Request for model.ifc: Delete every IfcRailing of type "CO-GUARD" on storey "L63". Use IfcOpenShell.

First a look at what the model holds.

```python
import ifcopenshell
import ifcopenshell.util.element

model = ifcopenshell.open("model.ifc")
print(model.schema)
storey = next(s for s in model.by_type("IfcBuildingStorey") if s.Name == "L63")
railings = [e for e in ifcopenshell.util.element.get_decomposition(storey) if e.is_a("IfcRailing")]
seen = {}
for e in railings:
    element_type = ifcopenshell.util.element.get_type(e)
    name = element_type.Name if element_type not in (None, e) else None
    seen[name] = seen.get(name, 0) + 1
for name, count in sorted(seen.items(), key=str):
    print(count, "x", name)
```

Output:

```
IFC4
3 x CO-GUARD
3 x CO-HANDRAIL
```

```python
import ifcopenshell
import ifcopenshell.api.root
import ifcopenshell.util.element

model = ifcopenshell.open("model.ifc")

storey = next(s for s in model.by_type("IfcBuildingStorey") if s.Name == "L63")
railings = [e for e in ifcopenshell.util.element.get_decomposition(storey) if e.is_a("IfcRailing")]
targets = [e for e in railings if (t := ifcopenshell.util.element.get_type(e)) not in (None, e) and t.Name == "CO-GUARD"]

for e in targets:
    ifcopenshell.api.root.remove_product(model, product=e)
print(len(targets), "removed")

model.write("model_updated.ifc")
```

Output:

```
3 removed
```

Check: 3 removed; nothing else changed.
